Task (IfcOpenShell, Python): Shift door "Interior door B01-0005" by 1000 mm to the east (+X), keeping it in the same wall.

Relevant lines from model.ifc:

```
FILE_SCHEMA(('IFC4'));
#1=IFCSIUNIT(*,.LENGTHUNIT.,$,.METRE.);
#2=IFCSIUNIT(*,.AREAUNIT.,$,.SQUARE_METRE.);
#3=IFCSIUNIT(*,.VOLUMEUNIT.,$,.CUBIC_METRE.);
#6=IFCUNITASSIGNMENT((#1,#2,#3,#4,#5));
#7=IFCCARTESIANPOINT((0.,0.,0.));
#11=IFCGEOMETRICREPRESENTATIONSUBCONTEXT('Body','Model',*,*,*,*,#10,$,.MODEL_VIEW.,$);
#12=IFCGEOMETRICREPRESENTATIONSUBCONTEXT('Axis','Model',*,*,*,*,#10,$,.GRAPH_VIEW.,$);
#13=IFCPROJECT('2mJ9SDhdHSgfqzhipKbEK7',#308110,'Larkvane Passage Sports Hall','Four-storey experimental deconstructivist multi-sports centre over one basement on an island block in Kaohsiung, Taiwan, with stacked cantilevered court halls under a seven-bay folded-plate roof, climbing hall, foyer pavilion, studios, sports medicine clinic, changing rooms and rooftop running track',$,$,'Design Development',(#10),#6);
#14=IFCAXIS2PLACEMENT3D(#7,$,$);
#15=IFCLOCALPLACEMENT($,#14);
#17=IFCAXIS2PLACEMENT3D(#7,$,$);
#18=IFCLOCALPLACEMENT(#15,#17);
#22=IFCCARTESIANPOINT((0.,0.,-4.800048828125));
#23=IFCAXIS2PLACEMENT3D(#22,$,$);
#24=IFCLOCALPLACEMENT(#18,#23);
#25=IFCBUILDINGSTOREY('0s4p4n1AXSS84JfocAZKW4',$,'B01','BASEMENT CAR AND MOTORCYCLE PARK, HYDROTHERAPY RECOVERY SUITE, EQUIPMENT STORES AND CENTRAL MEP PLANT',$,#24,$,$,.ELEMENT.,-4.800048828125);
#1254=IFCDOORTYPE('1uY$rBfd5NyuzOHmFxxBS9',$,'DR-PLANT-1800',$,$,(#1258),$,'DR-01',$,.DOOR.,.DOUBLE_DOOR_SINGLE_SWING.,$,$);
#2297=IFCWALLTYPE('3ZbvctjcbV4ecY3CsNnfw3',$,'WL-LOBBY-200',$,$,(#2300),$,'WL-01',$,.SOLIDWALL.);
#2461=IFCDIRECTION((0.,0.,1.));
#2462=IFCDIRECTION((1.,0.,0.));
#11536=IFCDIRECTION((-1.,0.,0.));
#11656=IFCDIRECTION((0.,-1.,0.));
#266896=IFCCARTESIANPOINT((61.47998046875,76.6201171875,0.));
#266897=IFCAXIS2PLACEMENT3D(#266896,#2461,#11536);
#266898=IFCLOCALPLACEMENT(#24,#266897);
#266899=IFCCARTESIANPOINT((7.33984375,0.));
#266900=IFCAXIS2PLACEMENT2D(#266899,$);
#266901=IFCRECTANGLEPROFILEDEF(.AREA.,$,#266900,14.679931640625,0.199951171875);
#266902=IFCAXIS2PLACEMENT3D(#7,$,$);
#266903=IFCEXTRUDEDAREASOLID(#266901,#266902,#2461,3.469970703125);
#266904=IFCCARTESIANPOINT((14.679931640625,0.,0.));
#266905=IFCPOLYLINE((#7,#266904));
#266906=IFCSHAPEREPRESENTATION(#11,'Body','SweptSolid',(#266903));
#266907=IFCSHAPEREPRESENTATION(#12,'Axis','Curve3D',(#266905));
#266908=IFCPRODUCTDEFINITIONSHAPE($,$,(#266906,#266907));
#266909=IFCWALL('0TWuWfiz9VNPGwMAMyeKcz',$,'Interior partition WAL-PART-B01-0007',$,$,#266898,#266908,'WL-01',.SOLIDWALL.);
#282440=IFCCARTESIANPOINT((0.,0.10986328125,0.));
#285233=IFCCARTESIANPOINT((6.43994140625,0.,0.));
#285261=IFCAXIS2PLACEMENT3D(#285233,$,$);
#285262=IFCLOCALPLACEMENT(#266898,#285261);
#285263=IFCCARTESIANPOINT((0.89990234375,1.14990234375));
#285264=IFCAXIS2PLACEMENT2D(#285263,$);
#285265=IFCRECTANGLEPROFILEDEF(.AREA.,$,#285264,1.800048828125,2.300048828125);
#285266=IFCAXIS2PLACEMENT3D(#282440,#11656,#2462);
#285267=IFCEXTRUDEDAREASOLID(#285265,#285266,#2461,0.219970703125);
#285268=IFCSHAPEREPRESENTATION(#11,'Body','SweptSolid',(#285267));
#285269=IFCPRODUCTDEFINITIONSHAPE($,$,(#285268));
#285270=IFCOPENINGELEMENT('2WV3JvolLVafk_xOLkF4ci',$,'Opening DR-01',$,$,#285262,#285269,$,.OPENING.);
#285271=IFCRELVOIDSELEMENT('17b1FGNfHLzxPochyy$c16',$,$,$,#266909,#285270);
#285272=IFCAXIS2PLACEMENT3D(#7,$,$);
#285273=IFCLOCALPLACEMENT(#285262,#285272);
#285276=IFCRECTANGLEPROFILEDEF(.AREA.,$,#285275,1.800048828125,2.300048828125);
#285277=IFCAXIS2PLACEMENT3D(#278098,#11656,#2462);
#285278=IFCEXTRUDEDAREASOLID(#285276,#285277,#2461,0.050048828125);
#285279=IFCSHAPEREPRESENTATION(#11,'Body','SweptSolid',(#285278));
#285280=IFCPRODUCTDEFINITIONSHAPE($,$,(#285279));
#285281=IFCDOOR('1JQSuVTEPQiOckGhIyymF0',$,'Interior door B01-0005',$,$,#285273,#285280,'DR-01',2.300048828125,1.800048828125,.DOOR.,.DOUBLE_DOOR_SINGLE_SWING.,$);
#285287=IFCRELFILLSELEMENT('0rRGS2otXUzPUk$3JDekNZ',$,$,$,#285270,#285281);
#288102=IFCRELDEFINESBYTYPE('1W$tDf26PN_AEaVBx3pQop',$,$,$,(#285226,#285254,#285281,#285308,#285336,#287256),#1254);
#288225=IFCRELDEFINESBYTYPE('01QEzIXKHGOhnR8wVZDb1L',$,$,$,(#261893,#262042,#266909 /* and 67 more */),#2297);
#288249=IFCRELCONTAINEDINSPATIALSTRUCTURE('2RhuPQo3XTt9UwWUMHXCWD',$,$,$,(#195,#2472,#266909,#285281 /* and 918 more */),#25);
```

```python
import ifcopenshell
import ifcopenshell.api.geometry
import ifcopenshell.util.placement
import ifcopenshell.util.unit

model = ifcopenshell.open("model.ifc")
unit_scale = ifcopenshell.util.unit.calculate_unit_scale(model)

door = model.by_id(285281)
opening = door.FillsVoids[0].RelatingOpeningElement
wall = opening.VoidsElements[0].RelatingBuildingElement

wall_matrix = ifcopenshell.util.placement.get_local_placement(wall.ObjectPlacement)
shift = wall_matrix[:3, 0] * -1 / unit_scale
before = ifcopenshell.util.placement.get_local_placement(door.ObjectPlacement)[:3, 3].copy()

# The door is placed relative to its opening, so it follows when the opening moves.
matrix = ifcopenshell.util.placement.get_local_placement(opening.ObjectPlacement)
matrix[:3, 3] += shift
ifcopenshell.api.geometry.edit_object_placement(
    model, product=opening, matrix=matrix, is_si=False, should_transform_children=True
)

after = ifcopenshell.util.placement.get_local_placement(door.ObjectPlacement)[:3, 3]
print("door moved by", (after - before).round(3) + 0.0)

model.write("model_updated.ifc")
```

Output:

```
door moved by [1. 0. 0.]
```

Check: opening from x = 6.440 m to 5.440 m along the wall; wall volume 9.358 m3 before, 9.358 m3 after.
